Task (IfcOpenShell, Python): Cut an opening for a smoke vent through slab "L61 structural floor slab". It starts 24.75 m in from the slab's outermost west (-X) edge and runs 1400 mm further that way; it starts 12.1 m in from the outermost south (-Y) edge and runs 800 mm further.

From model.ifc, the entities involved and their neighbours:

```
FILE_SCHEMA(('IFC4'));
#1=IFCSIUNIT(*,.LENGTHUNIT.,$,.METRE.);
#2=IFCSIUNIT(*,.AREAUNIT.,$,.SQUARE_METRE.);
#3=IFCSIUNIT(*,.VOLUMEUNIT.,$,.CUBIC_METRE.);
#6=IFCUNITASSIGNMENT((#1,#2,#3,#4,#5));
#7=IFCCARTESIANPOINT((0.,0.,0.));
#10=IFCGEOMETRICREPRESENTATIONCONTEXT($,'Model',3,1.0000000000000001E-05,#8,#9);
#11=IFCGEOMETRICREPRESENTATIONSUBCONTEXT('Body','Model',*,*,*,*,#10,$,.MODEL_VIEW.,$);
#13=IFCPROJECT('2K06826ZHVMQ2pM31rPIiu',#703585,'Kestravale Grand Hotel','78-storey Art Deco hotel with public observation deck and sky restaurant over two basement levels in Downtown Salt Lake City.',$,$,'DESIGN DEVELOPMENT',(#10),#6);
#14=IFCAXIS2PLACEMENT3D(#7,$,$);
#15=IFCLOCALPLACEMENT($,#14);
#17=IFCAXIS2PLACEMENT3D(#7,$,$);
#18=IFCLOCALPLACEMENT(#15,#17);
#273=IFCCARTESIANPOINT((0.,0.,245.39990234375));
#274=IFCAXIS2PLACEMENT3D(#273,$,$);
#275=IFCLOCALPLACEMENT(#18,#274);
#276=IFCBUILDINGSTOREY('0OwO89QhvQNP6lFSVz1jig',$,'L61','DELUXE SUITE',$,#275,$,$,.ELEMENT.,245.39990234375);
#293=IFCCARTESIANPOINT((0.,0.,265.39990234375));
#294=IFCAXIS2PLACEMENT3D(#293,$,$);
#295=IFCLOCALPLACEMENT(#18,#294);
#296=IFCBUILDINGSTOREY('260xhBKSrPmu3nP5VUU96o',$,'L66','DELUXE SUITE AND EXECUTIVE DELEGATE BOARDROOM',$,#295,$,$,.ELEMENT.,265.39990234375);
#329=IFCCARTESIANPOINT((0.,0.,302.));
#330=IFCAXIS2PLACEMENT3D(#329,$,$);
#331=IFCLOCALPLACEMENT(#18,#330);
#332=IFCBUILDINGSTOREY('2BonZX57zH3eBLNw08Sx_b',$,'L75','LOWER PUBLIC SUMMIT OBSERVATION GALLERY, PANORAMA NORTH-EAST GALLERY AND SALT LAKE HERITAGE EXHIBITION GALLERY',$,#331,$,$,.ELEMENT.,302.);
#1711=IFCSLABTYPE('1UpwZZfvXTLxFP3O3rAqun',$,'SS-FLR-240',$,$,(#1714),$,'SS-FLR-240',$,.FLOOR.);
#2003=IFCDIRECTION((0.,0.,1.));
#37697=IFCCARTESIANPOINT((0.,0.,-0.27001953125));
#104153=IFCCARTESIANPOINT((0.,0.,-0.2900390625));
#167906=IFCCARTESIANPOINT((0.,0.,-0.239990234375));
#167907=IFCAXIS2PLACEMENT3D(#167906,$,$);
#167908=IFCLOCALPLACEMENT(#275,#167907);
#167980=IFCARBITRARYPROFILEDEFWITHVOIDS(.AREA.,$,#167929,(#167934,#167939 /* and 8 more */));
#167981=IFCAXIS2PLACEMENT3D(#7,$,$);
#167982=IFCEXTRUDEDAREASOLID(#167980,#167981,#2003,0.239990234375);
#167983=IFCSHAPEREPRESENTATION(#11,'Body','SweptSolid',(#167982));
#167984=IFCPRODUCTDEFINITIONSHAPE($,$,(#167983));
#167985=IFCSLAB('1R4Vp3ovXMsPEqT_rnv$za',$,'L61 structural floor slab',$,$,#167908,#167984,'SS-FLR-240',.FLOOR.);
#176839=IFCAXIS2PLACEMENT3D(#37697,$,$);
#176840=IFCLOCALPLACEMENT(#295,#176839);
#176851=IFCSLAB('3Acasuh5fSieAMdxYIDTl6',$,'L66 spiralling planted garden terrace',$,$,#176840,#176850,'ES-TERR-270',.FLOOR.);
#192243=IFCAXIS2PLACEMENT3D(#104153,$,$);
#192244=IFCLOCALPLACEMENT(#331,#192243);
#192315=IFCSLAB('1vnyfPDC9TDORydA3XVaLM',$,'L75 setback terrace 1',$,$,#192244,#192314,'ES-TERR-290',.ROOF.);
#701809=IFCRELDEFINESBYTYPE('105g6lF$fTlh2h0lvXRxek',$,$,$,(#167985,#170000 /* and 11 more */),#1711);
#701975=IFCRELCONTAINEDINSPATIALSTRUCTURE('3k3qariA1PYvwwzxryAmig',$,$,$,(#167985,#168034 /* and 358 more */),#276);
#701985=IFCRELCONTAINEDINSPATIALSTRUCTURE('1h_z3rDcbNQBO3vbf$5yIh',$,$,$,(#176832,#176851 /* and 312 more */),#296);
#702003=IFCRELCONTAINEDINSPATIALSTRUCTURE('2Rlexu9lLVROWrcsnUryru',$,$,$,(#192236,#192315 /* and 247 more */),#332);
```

```python
import numpy as np
import ifcopenshell
import ifcopenshell.api.feature
import ifcopenshell.api.geometry
import ifcopenshell.api.root
import ifcopenshell.geom
import ifcopenshell.util.placement
import ifcopenshell.util.representation
import ifcopenshell.util.shape
import ifcopenshell.util.unit

model = ifcopenshell.open("model.ifc")
unit_scale = ifcopenshell.util.unit.calculate_unit_scale(model)
settings = ifcopenshell.geom.settings()


def volume(element):
    """Net volume in cubic metres, openings subtracted."""
    shape = ifcopenshell.geom.create_shape(settings, element)
    return ifcopenshell.util.shape.get_volume(shape.geometry)


slab = model.by_guid("1R4Vp3ovXMsPEqT_rnv$za")
before = volume(slab)

# Extent in the slab's own axes, in metres. The edges named are its -X and -Y sides.
slab_shape = ifcopenshell.geom.create_shape(settings, slab)
vertices = ifcopenshell.util.shape.get_vertices(slab_shape.geometry)
x_min, y_min, bottom = vertices.min(axis=0)
top = vertices[:, 2].max()

opening = ifcopenshell.api.root.create_entity(model, ifc_class="IfcOpeningElement", name="Smoke vent opening", predefined_type="OPENING")
context = ifcopenshell.util.representation.get_context(model, "Model", "Body", "MODEL_VIEW")
width, depth = 1.4, 0.8
outline = [(0.0, 0.0), (width, 0.0), (width, depth), (0.0, depth), (0.0, 0.0)]
# Overshoot both faces by 50 mm so the cut is clean.
shape = ifcopenshell.api.geometry.add_slab_representation(
    model, context=context, depth=top - bottom + 0.1, polyline=outline
)
ifcopenshell.api.geometry.assign_representation(model, product=opening, representation=shape)

matrix = ifcopenshell.util.placement.get_local_placement(slab.ObjectPlacement)
matrix[:, 3] = matrix @ np.append(np.array([x_min + 24.75, y_min + 12.1, bottom - 0.05]) / unit_scale, 1.0)
ifcopenshell.api.geometry.edit_object_placement(model, product=opening, matrix=matrix, is_si=False)
ifcopenshell.api.feature.add_feature(model, feature=opening, element=slab)

after = volume(slab)

print(f"slab volume {before:.3f} -> {after:.3f} m3")

model.write("model_updated.ifc")
```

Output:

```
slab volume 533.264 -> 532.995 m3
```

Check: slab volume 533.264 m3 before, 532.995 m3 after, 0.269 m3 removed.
